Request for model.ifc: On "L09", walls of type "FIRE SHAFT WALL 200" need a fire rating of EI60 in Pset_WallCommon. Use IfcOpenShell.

First a look at what the model holds.

```python
import ifcopenshell
import ifcopenshell.util.element

model = ifcopenshell.open("model.ifc")
print(model.schema)
storey = next(s for s in model.by_type("IfcBuildingStorey") if s.Name == "L09")
walls = [e for e in ifcopenshell.util.element.get_decomposition(storey) if e.is_a("IfcWall")]
seen = {}
for e in walls:
    element_type = ifcopenshell.util.element.get_type(e)
    key = (element_type.Name if element_type != e and element_type else None, ifcopenshell.util.element.get_pset(e, "Pset_WallCommon", "FireRating"))
    seen[key] = seen.get(key, 0) + 1
for (name, value), count in sorted(seen.items(), key=str):
    print(count, "x", name, "|", value)
```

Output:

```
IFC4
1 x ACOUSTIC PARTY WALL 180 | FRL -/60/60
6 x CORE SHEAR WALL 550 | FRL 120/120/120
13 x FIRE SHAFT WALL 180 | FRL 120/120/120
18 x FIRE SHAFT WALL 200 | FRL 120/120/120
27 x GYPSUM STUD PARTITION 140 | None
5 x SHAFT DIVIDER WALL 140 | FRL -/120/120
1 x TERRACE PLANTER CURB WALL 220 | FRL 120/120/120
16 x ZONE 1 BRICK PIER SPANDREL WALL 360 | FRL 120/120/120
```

```python
import ifcopenshell
import ifcopenshell.api.pset
import ifcopenshell.util.element

model = ifcopenshell.open("model.ifc")

storey = next(s for s in model.by_type("IfcBuildingStorey") if s.Name == "L09")
walls = [e for e in ifcopenshell.util.element.get_decomposition(storey) if e.is_a("IfcWall")]

count = 0
for e in walls:
    element_type = ifcopenshell.util.element.get_type(e)
    if element_type in (None, e) or element_type.Name != "FIRE SHAFT WALL 200":
        continue
    # add_pset returns the element's existing set when there is one.
    pset = ifcopenshell.api.pset.add_pset(model, product=e, name="Pset_WallCommon")
    ifcopenshell.api.pset.edit_pset(model, pset=pset, properties={"FireRating": "EI60"})
    count += 1

print(count, "walls updated")

model.write("model_updated.ifc")
```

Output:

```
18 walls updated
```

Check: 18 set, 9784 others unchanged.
